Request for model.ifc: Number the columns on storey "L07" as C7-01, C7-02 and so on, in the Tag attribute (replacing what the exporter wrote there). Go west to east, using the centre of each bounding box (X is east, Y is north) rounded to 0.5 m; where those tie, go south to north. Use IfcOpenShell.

First a look at what the model holds.

```python
import ifcopenshell
import ifcopenshell.util.element
import ifcopenshell.util.placement

model = ifcopenshell.open("model.ifc")
print(model.schema)
storey = next(s for s in model.by_type("IfcBuildingStorey") if s.Name == "L07")
columns = [e for e in ifcopenshell.util.element.get_decomposition(storey) if e.is_a("IfcColumn")]
for e in sorted(columns, key=lambda e: e.id()):
    origin = ifcopenshell.util.placement.get_local_placement(e.ObjectPlacement)[:3, 3]
    print(e.id(), e.Tag, e.Name, origin.round(2) + 0.0, sep=" | ")
```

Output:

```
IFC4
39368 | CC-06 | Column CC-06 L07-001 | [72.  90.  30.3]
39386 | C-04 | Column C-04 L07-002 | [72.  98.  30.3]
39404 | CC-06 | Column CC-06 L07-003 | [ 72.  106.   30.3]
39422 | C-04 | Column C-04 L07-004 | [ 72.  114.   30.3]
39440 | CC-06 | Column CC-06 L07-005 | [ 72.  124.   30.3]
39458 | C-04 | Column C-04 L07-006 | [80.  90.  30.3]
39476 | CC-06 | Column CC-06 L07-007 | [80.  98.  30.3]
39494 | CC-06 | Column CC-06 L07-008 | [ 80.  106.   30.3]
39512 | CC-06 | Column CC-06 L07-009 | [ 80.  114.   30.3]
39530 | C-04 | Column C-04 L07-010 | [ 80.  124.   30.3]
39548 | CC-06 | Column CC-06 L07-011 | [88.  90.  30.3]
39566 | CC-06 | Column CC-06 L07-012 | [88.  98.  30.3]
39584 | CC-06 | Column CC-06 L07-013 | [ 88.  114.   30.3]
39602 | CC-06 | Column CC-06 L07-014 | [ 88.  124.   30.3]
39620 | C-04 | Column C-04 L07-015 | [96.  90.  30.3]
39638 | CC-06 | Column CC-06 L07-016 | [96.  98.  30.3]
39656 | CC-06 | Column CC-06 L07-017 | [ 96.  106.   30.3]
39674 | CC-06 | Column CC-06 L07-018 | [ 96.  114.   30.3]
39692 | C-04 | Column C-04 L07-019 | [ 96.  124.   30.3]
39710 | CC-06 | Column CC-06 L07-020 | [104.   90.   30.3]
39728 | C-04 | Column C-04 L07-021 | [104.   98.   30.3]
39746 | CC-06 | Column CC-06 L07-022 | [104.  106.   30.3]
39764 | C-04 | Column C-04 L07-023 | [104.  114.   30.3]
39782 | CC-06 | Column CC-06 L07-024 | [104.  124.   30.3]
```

```python
import ifcopenshell
import ifcopenshell.geom
import ifcopenshell.util.element
import ifcopenshell.util.shape

model = ifcopenshell.open("model.ifc")
settings = ifcopenshell.geom.settings()
settings.set("use-world-coords", True)


def centre(element):
    shape = ifcopenshell.geom.create_shape(settings, element)
    return ifcopenshell.util.shape.get_bbox_centroid(shape.geometry)


storey = next(s for s in model.by_type("IfcBuildingStorey") if s.Name == "L07")
columns = [e for e in ifcopenshell.util.element.get_decomposition(storey) if e.is_a("IfcColumn")]

# Insertion points can sit at a corner or the storey origin, so sort by the geometry (in metres).
centres = {e: centre(e) for e in columns}
columns.sort(key=lambda e: (round(centres[e][0] / 0.5), centres[e][1]))

for i, e in enumerate(columns, start=1):
    number = f"C7-{i:02d}"
    e.Tag = number
    print(e.id(), number)

model.write("model_updated.ifc")
```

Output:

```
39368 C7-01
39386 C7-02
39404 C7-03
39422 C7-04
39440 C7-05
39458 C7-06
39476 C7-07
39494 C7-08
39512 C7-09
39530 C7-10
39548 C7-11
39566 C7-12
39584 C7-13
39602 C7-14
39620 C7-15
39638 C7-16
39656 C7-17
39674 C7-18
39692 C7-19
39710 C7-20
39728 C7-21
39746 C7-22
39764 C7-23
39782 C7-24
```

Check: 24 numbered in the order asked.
